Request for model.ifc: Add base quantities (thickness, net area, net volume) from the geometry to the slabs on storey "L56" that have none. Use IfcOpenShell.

First a look at what the model holds.

```python
import ifcopenshell
import ifcopenshell.util.element
import ifcopenshell.util.unit

model = ifcopenshell.open("model.ifc")
print(model.schema)
for unit_type in ("LENGTHUNIT", "AREAUNIT", "VOLUMEUNIT"):
    print(unit_type, ifcopenshell.util.unit.calculate_unit_scale(model, unit_type))
storey = next(s for s in model.by_type("IfcBuildingStorey") if s.Name == "L56")
slabs = [e for e in ifcopenshell.util.element.get_decomposition(storey) if e.is_a("IfcSlab")]
for e in sorted(slabs, key=lambda e: e.id()):
    print(e.id(), e.is_a(), e.Name, list(ifcopenshell.util.element.get_psets(e, qtos_only=True)), sep=" | ")
```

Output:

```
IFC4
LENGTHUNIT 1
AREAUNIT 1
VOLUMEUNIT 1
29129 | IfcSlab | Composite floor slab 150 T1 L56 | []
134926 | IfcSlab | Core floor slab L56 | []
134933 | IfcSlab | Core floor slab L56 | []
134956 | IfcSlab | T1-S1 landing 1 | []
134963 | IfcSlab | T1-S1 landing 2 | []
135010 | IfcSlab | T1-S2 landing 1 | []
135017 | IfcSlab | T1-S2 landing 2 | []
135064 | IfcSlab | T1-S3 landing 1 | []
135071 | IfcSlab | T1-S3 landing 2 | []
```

```python
import ifcopenshell
import ifcopenshell.api.pset
import ifcopenshell.geom
import ifcopenshell.util.element
import ifcopenshell.util.shape
import ifcopenshell.util.unit

model = ifcopenshell.open("model.ifc")
unit_scale = ifcopenshell.util.unit.calculate_unit_scale(model)
area_scale = ifcopenshell.util.unit.calculate_unit_scale(model, "AREAUNIT")
volume_scale = ifcopenshell.util.unit.calculate_unit_scale(model, "VOLUMEUNIT")
settings = ifcopenshell.geom.settings()

storey = next(s for s in model.by_type("IfcBuildingStorey") if s.Name == "L56")
slabs = [e for e in ifcopenshell.util.element.get_decomposition(storey) if e.is_a("IfcSlab")]

for e in sorted(slabs, key=lambda e: e.id()):
    if ifcopenshell.util.element.get_psets(e, qtos_only=True, should_inherit=False):
        continue
    # Geometry comes back in metres, in the element's own axes.
    shape = ifcopenshell.geom.create_shape(settings, e)
    values = {
        "Width": ifcopenshell.util.shape.get_z(shape.geometry) / unit_scale,
        "NetArea": ifcopenshell.util.shape.get_footprint_area(shape.geometry) / area_scale,
        "NetVolume": ifcopenshell.util.shape.get_volume(shape.geometry) / volume_scale,
    }
    qto = ifcopenshell.api.pset.add_qto(model, product=e, name="Qto_SlabBaseQuantities")
    ifcopenshell.api.pset.edit_qto(model, qto=qto, properties=values)
    print(e.id(), {k: round(v, 3) for k, v in values.items()})

model.write("model_rev.ifc")
```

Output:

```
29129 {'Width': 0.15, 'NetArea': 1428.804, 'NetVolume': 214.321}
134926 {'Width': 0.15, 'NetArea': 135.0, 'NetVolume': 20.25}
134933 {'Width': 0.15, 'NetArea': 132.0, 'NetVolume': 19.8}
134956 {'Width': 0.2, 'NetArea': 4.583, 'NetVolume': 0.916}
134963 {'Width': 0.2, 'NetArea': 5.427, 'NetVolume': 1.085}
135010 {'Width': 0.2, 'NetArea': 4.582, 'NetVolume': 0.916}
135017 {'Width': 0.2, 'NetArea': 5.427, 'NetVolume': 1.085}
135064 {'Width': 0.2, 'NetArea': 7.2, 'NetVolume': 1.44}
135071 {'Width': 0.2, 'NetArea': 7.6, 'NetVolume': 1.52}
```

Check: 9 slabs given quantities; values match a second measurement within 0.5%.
